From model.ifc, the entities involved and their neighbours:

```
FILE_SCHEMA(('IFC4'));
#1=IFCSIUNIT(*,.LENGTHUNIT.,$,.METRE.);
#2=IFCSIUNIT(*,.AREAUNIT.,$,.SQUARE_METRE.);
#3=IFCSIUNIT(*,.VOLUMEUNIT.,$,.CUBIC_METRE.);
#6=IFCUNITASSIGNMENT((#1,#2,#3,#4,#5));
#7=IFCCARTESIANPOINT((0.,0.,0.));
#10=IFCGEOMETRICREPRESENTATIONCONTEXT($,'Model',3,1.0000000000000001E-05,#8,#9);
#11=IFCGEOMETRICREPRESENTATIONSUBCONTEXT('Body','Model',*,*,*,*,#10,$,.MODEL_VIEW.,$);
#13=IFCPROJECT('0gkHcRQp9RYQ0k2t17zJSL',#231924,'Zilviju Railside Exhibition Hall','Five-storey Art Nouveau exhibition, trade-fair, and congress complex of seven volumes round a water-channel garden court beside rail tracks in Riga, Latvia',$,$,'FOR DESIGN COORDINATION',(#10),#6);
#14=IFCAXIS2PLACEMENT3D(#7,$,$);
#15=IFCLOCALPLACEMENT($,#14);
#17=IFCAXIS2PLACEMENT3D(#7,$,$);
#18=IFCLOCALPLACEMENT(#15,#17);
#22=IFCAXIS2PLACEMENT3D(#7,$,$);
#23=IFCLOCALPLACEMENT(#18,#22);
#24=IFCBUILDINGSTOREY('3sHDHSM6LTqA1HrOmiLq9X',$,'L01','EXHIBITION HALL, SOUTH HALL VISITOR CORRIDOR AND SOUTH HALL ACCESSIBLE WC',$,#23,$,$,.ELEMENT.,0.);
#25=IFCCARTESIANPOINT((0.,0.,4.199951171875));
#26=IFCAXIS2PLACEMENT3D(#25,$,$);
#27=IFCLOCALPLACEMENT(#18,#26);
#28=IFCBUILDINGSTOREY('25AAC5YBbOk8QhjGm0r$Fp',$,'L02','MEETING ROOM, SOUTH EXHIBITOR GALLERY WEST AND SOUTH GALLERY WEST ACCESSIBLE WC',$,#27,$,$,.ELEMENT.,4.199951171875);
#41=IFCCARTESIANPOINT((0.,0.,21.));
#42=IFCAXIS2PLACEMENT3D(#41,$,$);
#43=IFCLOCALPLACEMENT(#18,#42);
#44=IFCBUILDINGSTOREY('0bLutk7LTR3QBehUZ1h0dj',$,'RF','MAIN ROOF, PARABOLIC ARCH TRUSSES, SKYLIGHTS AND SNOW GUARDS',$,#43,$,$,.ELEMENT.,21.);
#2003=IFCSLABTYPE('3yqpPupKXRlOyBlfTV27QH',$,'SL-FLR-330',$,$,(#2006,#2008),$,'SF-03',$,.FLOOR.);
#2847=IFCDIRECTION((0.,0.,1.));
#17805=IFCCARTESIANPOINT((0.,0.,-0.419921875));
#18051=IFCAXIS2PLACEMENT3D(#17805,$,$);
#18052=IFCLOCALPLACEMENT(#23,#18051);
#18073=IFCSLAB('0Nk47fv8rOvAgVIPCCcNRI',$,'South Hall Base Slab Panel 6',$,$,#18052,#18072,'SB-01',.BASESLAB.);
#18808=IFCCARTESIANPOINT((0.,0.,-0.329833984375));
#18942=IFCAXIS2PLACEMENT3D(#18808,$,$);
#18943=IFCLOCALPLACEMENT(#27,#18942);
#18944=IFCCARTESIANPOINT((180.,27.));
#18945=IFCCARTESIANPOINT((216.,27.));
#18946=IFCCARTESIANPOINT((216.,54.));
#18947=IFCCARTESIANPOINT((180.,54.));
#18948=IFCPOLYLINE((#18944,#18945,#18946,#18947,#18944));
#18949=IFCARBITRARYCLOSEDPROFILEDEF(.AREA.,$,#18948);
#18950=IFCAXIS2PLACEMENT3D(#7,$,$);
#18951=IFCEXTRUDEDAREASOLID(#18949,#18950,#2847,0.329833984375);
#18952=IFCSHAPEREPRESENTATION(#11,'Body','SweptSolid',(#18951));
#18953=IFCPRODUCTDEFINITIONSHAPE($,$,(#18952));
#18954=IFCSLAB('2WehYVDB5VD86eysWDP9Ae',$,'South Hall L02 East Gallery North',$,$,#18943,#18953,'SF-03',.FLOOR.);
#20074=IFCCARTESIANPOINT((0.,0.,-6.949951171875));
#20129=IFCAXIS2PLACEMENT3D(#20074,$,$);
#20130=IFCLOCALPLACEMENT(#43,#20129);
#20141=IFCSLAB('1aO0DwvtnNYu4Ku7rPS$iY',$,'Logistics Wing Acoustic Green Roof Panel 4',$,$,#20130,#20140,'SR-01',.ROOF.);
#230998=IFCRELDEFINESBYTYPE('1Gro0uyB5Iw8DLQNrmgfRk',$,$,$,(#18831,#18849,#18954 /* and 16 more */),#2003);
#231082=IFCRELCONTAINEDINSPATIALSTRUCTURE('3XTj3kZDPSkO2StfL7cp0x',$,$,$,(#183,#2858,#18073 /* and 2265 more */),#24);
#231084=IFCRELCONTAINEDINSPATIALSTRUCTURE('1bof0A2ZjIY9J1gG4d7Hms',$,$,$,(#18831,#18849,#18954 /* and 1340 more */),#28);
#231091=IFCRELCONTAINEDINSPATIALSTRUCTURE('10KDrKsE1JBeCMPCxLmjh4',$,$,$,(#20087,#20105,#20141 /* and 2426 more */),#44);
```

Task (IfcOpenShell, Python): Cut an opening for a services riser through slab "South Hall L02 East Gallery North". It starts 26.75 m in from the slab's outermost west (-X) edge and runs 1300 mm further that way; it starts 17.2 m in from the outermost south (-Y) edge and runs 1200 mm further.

```python
import numpy as np
import ifcopenshell
import ifcopenshell.api.feature
import ifcopenshell.api.geometry
import ifcopenshell.api.root
import ifcopenshell.geom
import ifcopenshell.util.placement
import ifcopenshell.util.representation
import ifcopenshell.util.shape
import ifcopenshell.util.unit

model = ifcopenshell.open("model.ifc")
unit_scale = ifcopenshell.util.unit.calculate_unit_scale(model)
settings = ifcopenshell.geom.settings()


def volume(element):
    """Net volume in cubic metres, openings subtracted."""
    shape = ifcopenshell.geom.create_shape(settings, element)
    return ifcopenshell.util.shape.get_volume(shape.geometry)


slab = model.by_id(18954)
before = volume(slab)

# Extent in the slab's own axes, in metres. The edges named are its -X and -Y sides.
slab_shape = ifcopenshell.geom.create_shape(settings, slab)
vertices = ifcopenshell.util.shape.get_vertices(slab_shape.geometry)
x_min, y_min, bottom = vertices.min(axis=0)
top = vertices[:, 2].max()

opening = ifcopenshell.api.root.create_entity(model, ifc_class="IfcOpeningElement", name="Services riser opening", predefined_type="OPENING")
context = ifcopenshell.util.representation.get_context(model, "Model", "Body", "MODEL_VIEW")
width, depth = 1.3, 1.2
outline = [(0.0, 0.0), (width, 0.0), (width, depth), (0.0, depth), (0.0, 0.0)]
# Overshoot both faces by 50 mm so the cut is clean.
shape = ifcopenshell.api.geometry.add_slab_representation(
    model, context=context, depth=top - bottom + 0.1, polyline=outline
)
ifcopenshell.api.geometry.assign_representation(model, product=opening, representation=shape)

matrix = ifcopenshell.util.placement.get_local_placement(slab.ObjectPlacement)
matrix[:, 3] = matrix @ np.append(np.array([x_min + 26.75, y_min + 17.2, bottom - 0.05]) / unit_scale, 1.0)
ifcopenshell.api.geometry.edit_object_placement(model, product=opening, matrix=matrix, is_si=False)
ifcopenshell.api.feature.add_feature(model, feature=opening, element=slab)

after = volume(slab)

print(f"slab volume {before:.3f} -> {after:.3f} m3")

model.write("model_edited.ifc")
```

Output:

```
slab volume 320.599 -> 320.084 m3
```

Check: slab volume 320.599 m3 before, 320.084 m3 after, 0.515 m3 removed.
